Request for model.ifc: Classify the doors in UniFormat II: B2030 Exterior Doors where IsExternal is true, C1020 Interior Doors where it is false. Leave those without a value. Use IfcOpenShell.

First a look at what the model holds.

```python
import ifcopenshell
import ifcopenshell.util.element

model = ifcopenshell.open("model.ifc")
print(model.schema)
print("classifications:", [c.Name for c in model.by_type("IfcClassification")])
values = [ifcopenshell.util.element.get_pset(e, "Pset_DoorCommon", "IsExternal") for e in model.by_type("IfcDoor")]
for value in (True, False, None):
    print("IsExternal", value, values.count(value))
```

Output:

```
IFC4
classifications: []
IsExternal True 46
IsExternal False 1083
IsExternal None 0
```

```python
import ifcopenshell
import ifcopenshell.api.classification
import ifcopenshell.util.element

model = ifcopenshell.open("model.ifc")

system = ifcopenshell.api.classification.add_classification(model, classification="UniFormat II")

doors = model.by_type("IfcDoor")
external = {e: ifcopenshell.util.element.get_pset(e, "Pset_DoorCommon", "IsExternal") for e in doors}
for flag, code, name in ((True, "B2030", "Exterior Doors"), (False, "C1020", "Interior Doors")):
    products = [e for e in doors if external[e] is flag]
    ifcopenshell.api.classification.add_reference(
        model, products=products, classification=system, identification=code, name=name
    )
    print(code, len(products))

model.write("model_updated.ifc")
```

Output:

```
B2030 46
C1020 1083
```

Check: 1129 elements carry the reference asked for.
